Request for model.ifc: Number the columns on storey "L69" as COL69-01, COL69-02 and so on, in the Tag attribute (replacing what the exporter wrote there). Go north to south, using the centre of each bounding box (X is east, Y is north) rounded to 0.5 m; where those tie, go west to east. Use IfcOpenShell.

First a look at what the model holds.

```python
import ifcopenshell
import ifcopenshell.util.element
import ifcopenshell.util.placement

model = ifcopenshell.open("model.ifc")
print(model.schema)
storey = next(s for s in model.by_type("IfcBuildingStorey") if s.Name == "L69")
columns = [e for e in ifcopenshell.util.element.get_decomposition(storey) if e.is_a("IfcColumn")]
for e in sorted(columns, key=lambda e: e.id()):
    origin = ifcopenshell.util.placement.get_local_placement(e.ObjectPlacement)[:3, 3]
    print(e.id(), e.Tag, e.Name, origin.round(2) + 0.0, sep=" | ")
```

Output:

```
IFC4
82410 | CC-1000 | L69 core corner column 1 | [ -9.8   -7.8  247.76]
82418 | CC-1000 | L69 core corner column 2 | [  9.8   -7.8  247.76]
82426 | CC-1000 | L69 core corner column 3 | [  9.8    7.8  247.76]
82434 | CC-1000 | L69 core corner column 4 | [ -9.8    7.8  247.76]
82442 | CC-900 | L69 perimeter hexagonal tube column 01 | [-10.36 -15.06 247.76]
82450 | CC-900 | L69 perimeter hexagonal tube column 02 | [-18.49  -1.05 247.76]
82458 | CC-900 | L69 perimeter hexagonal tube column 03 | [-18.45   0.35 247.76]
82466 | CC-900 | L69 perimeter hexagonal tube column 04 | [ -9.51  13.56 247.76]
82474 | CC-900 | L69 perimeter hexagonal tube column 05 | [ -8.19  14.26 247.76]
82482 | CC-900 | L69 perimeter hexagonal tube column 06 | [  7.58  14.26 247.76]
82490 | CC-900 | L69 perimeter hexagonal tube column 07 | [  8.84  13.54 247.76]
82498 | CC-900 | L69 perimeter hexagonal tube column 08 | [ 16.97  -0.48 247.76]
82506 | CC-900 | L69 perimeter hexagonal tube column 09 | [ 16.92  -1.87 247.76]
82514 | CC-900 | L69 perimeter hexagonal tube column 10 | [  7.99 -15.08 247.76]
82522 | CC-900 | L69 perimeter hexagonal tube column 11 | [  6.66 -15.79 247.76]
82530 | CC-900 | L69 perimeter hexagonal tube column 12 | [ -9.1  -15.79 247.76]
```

```python
import ifcopenshell
import ifcopenshell.geom
import ifcopenshell.util.element
import ifcopenshell.util.shape

model = ifcopenshell.open("model.ifc")
settings = ifcopenshell.geom.settings()
settings.set("use-world-coords", True)


def centre(element):
    shape = ifcopenshell.geom.create_shape(settings, element)
    return ifcopenshell.util.shape.get_bbox_centroid(shape.geometry)


storey = next(s for s in model.by_type("IfcBuildingStorey") if s.Name == "L69")
columns = [e for e in ifcopenshell.util.element.get_decomposition(storey) if e.is_a("IfcColumn")]

# Insertion points can sit at a corner or the storey origin, so sort by the geometry (in metres).
centres = {e: centre(e) for e in columns}
columns.sort(key=lambda e: (-round(centres[e][1] / 0.5), centres[e][0]))

for i, e in enumerate(columns, start=1):
    number = f"COL69-{i:02d}"
    e.Tag = number
    print(e.id(), number)

model.write("model-out.ifc")
```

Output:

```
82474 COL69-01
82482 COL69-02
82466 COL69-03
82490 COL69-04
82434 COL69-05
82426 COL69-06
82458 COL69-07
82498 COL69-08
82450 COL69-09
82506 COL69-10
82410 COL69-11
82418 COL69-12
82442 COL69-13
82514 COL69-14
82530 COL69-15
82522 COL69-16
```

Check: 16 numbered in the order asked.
